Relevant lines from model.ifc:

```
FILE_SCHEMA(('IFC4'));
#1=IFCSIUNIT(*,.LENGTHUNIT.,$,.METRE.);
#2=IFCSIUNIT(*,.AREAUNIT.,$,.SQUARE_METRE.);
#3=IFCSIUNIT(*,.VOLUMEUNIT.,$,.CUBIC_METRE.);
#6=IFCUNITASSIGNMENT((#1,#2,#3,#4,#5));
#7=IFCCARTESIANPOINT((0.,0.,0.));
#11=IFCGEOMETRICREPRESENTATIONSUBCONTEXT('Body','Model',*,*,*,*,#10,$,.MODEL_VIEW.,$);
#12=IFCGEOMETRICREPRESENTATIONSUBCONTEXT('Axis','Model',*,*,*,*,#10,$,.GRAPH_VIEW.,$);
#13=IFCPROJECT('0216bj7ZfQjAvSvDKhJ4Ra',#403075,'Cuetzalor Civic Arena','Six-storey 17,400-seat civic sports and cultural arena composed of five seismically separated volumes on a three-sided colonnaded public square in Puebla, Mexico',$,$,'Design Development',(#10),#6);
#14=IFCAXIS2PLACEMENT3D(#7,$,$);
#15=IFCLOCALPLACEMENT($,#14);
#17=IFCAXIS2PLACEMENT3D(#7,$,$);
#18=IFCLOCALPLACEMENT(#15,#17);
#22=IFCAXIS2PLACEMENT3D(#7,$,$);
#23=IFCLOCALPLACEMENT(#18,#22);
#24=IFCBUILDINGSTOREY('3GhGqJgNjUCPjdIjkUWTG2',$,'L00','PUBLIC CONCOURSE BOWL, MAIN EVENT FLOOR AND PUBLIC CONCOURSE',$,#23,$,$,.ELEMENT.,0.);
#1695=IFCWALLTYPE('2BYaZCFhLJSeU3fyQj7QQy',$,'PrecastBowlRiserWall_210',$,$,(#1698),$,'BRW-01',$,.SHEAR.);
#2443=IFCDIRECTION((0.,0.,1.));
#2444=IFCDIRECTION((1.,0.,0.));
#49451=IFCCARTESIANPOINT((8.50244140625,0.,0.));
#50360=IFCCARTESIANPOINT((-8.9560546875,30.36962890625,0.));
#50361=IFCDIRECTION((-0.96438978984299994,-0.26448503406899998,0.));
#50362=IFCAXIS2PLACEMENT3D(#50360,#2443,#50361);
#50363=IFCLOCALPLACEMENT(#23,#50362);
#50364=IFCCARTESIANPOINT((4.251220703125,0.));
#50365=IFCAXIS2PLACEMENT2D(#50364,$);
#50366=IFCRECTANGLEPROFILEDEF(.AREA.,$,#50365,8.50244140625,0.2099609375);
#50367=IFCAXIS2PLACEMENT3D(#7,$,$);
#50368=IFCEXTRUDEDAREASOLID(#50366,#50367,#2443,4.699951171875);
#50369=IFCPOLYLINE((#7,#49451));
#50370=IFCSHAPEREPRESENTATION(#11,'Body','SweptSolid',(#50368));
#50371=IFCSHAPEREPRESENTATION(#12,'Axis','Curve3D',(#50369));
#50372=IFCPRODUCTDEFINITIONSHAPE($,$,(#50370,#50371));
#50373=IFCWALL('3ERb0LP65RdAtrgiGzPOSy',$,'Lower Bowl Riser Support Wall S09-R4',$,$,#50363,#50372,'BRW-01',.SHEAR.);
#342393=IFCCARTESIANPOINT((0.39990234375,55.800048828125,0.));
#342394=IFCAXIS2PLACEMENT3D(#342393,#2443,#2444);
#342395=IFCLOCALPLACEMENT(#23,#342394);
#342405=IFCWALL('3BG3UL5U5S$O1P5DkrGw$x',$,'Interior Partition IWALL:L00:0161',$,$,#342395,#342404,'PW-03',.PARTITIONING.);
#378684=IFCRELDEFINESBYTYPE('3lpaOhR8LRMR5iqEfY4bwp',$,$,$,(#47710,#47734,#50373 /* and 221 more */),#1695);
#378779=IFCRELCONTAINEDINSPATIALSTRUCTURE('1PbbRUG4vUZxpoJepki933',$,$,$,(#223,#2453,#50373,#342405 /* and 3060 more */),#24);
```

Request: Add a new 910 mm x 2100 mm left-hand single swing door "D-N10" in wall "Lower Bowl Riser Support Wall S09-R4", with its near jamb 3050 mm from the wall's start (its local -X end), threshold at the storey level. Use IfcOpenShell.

```python
import numpy as np
import ifcopenshell
import ifcopenshell.api.feature
import ifcopenshell.api.geometry
import ifcopenshell.api.root
import ifcopenshell.api.spatial
import ifcopenshell.geom
import ifcopenshell.util.element
import ifcopenshell.util.placement
import ifcopenshell.util.representation
import ifcopenshell.util.shape
import ifcopenshell.util.unit

model = ifcopenshell.open("model.ifc")
unit_scale = ifcopenshell.util.unit.calculate_unit_scale(model)
settings = ifcopenshell.geom.settings()


def volume(element):
    """Net volume in cubic metres, openings subtracted."""
    shape = ifcopenshell.geom.create_shape(settings, element)
    return ifcopenshell.util.shape.get_volume(shape.geometry)


wall = model.by_guid("3ERb0LP65RdAtrgiGzPOSy")
storey = ifcopenshell.util.element.get_container(wall, ifc_class="IfcBuildingStorey")
context = ifcopenshell.util.representation.get_context(model, "Model", "Body", "MODEL_VIEW")
before = volume(wall)

width, height, from_end, sill = 0.91, 2.1, 3.05, 0.0  # metres

# The wall runs along its own X axis, and the end named is its -X end.
wall_shape = ifcopenshell.geom.create_shape(settings, wall)
x, y, z = ifcopenshell.util.shape.get_vertices(wall_shape.geometry).T
start = x.min() + from_end
face, thickness = float(y.min()), float(y.max() - y.min())
wall_matrix = ifcopenshell.util.placement.get_local_placement(wall.ObjectPlacement)
level = ifcopenshell.util.placement.get_local_placement(storey.ObjectPlacement)[2, 3]


def in_wall(x, y):
    """Placement at x, y metres in the wall's axes, at sill height."""
    matrix = wall_matrix.copy()
    matrix[:, 3] = wall_matrix @ np.array([x / unit_scale, y / unit_scale, 0.0, 1.0])
    matrix[2, 3] = level + sill / unit_scale
    return matrix


# Opening: a box that overshoots both wall faces by 50 mm.
opening = ifcopenshell.api.root.create_entity(model, ifc_class="IfcOpeningElement", predefined_type="OPENING")
box = ifcopenshell.api.geometry.add_wall_representation(
    model, context=context, length=width, height=height, thickness=thickness + 0.1
)
ifcopenshell.api.geometry.assign_representation(model, product=opening, representation=box)
ifcopenshell.api.geometry.edit_object_placement(model, product=opening, matrix=in_wall(start, face - 0.05), is_si=False)
ifcopenshell.api.feature.add_feature(model, feature=opening, element=wall)

door = ifcopenshell.api.root.create_entity(model, ifc_class="IfcDoor", name="D-N10", predefined_type="DOOR")
door.OverallWidth, door.OverallHeight = width / unit_scale, height / unit_scale
door.OperationType = "SINGLE_SWING_LEFT"
body = ifcopenshell.api.geometry.add_door_representation(
    model,
    context=context,
    overall_width=door.OverallWidth,
    overall_height=door.OverallHeight,
    operation_type="SINGLE_SWING_LEFT",
    lining_properties={"LiningDepth": thickness / unit_scale, "ThresholdDepth": thickness / unit_scale},
)
ifcopenshell.api.geometry.assign_representation(model, product=door, representation=body)
ifcopenshell.api.spatial.assign_container(model, products=[door], relating_structure=storey)
ifcopenshell.api.feature.add_filling(model, opening=opening, element=door)

# The lining spans the wall, so the door starts at the wall face.
ifcopenshell.api.geometry.edit_object_placement(model, product=door, matrix=in_wall(start, face), is_si=False)

after = volume(wall)

print(f"wall volume {before:.3f} -> {after:.3f} m3")

model.write("model_updated.ifc")
```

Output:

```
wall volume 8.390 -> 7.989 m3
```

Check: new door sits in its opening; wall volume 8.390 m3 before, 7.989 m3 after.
